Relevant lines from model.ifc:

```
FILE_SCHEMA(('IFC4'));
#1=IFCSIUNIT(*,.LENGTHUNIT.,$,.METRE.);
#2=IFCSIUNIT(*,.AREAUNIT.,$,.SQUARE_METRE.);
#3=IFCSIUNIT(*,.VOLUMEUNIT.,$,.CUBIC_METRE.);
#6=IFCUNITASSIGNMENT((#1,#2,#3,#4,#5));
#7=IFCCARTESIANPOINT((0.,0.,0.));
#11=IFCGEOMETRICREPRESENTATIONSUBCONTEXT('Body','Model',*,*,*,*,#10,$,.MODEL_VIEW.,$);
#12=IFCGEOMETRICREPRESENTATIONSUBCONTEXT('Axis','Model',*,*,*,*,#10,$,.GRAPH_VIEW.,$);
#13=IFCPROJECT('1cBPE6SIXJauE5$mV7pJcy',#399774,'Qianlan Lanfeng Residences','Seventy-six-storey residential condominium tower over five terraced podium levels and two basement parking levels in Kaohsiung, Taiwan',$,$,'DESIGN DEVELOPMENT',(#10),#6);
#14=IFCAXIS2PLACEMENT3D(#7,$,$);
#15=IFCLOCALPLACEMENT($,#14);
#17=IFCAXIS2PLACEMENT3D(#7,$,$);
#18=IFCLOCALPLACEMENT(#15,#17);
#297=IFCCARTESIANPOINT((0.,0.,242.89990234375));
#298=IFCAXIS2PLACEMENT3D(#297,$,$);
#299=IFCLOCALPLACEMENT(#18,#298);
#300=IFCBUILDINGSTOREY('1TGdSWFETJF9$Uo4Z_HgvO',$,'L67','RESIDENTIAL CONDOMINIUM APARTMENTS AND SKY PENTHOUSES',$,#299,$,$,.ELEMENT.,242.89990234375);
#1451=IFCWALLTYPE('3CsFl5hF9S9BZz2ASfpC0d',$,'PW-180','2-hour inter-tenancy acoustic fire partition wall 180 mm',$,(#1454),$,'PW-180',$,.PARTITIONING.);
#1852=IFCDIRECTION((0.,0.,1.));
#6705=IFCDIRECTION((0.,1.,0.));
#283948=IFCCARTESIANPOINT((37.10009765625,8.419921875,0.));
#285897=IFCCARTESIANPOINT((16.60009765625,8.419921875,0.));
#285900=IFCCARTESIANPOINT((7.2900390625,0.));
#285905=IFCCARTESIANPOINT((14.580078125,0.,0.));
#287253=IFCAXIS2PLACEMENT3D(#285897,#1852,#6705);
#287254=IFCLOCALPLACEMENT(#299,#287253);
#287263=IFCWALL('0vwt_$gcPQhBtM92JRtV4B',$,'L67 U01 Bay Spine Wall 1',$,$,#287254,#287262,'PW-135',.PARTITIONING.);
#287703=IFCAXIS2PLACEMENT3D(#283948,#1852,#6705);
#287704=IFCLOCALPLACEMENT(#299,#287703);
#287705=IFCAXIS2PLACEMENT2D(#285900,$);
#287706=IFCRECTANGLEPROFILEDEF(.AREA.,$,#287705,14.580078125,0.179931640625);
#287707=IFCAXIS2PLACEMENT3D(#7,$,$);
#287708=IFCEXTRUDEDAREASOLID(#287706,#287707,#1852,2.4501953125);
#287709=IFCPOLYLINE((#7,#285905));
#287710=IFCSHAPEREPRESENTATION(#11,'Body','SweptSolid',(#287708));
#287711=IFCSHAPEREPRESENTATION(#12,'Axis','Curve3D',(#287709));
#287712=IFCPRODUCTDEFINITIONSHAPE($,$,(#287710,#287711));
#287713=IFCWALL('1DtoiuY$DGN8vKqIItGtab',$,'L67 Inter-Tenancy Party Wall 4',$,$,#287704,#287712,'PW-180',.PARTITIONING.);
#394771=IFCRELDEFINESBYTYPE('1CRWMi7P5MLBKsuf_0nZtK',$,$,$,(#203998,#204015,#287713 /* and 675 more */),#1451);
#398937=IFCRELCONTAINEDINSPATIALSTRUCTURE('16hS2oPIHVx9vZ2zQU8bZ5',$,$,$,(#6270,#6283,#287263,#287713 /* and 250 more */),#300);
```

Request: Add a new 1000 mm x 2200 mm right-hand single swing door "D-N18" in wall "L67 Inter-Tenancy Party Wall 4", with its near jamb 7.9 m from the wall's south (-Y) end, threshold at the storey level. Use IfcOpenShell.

```python
import numpy as np
import ifcopenshell
import ifcopenshell.api.feature
import ifcopenshell.api.geometry
import ifcopenshell.api.root
import ifcopenshell.api.spatial
import ifcopenshell.geom
import ifcopenshell.util.element
import ifcopenshell.util.placement
import ifcopenshell.util.representation
import ifcopenshell.util.shape
import ifcopenshell.util.unit

model = ifcopenshell.open("model.ifc")
unit_scale = ifcopenshell.util.unit.calculate_unit_scale(model)
settings = ifcopenshell.geom.settings()


def volume(element):
    """Net volume in cubic metres, openings subtracted."""
    shape = ifcopenshell.geom.create_shape(settings, element)
    return ifcopenshell.util.shape.get_volume(shape.geometry)


wall = model.by_guid("1DtoiuY$DGN8vKqIItGtab")
storey = ifcopenshell.util.element.get_container(wall, ifc_class="IfcBuildingStorey")
context = ifcopenshell.util.representation.get_context(model, "Model", "Body", "MODEL_VIEW")
before = volume(wall)

width, height, from_end, sill = 1, 2.2, 7.9, 0.0  # metres

# The wall runs along its own X axis, and the end named is its -X end.
wall_shape = ifcopenshell.geom.create_shape(settings, wall)
x, y, z = ifcopenshell.util.shape.get_vertices(wall_shape.geometry).T
start = x.min() + from_end
face, thickness = float(y.min()), float(y.max() - y.min())
wall_matrix = ifcopenshell.util.placement.get_local_placement(wall.ObjectPlacement)
level = ifcopenshell.util.placement.get_local_placement(storey.ObjectPlacement)[2, 3]


def in_wall(x, y):
    """Placement at x, y metres in the wall's axes, at sill height."""
    matrix = wall_matrix.copy()
    matrix[:, 3] = wall_matrix @ np.array([x / unit_scale, y / unit_scale, 0.0, 1.0])
    matrix[2, 3] = level + sill / unit_scale
    return matrix


# Opening: a box that overshoots both wall faces by 50 mm.
opening = ifcopenshell.api.root.create_entity(model, ifc_class="IfcOpeningElement", predefined_type="OPENING")
box = ifcopenshell.api.geometry.add_wall_representation(
    model, context=context, length=width, height=height, thickness=thickness + 0.1
)
ifcopenshell.api.geometry.assign_representation(model, product=opening, representation=box)
ifcopenshell.api.geometry.edit_object_placement(model, product=opening, matrix=in_wall(start, face - 0.05), is_si=False)
ifcopenshell.api.feature.add_feature(model, feature=opening, element=wall)

door = ifcopenshell.api.root.create_entity(model, ifc_class="IfcDoor", name="D-N18", predefined_type="DOOR")
door.OverallWidth, door.OverallHeight = width / unit_scale, height / unit_scale
door.OperationType = "SINGLE_SWING_RIGHT"
body = ifcopenshell.api.geometry.add_door_representation(
    model,
    context=context,
    overall_width=door.OverallWidth,
    overall_height=door.OverallHeight,
    operation_type="SINGLE_SWING_RIGHT",
    lining_properties={"LiningDepth": thickness / unit_scale, "ThresholdDepth": thickness / unit_scale},
)
ifcopenshell.api.geometry.assign_representation(model, product=door, representation=body)
ifcopenshell.api.spatial.assign_container(model, products=[door], relating_structure=storey)
ifcopenshell.api.feature.add_filling(model, opening=opening, element=door)

# The lining spans the wall, so the door starts at the wall face.
ifcopenshell.api.geometry.edit_object_placement(model, product=door, matrix=in_wall(start, face), is_si=False)

after = volume(wall)

print(f"wall volume {before:.3f} -> {after:.3f} m3")

model.write("model_edited.ifc")
```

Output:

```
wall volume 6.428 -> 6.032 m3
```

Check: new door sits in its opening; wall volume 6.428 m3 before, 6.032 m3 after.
